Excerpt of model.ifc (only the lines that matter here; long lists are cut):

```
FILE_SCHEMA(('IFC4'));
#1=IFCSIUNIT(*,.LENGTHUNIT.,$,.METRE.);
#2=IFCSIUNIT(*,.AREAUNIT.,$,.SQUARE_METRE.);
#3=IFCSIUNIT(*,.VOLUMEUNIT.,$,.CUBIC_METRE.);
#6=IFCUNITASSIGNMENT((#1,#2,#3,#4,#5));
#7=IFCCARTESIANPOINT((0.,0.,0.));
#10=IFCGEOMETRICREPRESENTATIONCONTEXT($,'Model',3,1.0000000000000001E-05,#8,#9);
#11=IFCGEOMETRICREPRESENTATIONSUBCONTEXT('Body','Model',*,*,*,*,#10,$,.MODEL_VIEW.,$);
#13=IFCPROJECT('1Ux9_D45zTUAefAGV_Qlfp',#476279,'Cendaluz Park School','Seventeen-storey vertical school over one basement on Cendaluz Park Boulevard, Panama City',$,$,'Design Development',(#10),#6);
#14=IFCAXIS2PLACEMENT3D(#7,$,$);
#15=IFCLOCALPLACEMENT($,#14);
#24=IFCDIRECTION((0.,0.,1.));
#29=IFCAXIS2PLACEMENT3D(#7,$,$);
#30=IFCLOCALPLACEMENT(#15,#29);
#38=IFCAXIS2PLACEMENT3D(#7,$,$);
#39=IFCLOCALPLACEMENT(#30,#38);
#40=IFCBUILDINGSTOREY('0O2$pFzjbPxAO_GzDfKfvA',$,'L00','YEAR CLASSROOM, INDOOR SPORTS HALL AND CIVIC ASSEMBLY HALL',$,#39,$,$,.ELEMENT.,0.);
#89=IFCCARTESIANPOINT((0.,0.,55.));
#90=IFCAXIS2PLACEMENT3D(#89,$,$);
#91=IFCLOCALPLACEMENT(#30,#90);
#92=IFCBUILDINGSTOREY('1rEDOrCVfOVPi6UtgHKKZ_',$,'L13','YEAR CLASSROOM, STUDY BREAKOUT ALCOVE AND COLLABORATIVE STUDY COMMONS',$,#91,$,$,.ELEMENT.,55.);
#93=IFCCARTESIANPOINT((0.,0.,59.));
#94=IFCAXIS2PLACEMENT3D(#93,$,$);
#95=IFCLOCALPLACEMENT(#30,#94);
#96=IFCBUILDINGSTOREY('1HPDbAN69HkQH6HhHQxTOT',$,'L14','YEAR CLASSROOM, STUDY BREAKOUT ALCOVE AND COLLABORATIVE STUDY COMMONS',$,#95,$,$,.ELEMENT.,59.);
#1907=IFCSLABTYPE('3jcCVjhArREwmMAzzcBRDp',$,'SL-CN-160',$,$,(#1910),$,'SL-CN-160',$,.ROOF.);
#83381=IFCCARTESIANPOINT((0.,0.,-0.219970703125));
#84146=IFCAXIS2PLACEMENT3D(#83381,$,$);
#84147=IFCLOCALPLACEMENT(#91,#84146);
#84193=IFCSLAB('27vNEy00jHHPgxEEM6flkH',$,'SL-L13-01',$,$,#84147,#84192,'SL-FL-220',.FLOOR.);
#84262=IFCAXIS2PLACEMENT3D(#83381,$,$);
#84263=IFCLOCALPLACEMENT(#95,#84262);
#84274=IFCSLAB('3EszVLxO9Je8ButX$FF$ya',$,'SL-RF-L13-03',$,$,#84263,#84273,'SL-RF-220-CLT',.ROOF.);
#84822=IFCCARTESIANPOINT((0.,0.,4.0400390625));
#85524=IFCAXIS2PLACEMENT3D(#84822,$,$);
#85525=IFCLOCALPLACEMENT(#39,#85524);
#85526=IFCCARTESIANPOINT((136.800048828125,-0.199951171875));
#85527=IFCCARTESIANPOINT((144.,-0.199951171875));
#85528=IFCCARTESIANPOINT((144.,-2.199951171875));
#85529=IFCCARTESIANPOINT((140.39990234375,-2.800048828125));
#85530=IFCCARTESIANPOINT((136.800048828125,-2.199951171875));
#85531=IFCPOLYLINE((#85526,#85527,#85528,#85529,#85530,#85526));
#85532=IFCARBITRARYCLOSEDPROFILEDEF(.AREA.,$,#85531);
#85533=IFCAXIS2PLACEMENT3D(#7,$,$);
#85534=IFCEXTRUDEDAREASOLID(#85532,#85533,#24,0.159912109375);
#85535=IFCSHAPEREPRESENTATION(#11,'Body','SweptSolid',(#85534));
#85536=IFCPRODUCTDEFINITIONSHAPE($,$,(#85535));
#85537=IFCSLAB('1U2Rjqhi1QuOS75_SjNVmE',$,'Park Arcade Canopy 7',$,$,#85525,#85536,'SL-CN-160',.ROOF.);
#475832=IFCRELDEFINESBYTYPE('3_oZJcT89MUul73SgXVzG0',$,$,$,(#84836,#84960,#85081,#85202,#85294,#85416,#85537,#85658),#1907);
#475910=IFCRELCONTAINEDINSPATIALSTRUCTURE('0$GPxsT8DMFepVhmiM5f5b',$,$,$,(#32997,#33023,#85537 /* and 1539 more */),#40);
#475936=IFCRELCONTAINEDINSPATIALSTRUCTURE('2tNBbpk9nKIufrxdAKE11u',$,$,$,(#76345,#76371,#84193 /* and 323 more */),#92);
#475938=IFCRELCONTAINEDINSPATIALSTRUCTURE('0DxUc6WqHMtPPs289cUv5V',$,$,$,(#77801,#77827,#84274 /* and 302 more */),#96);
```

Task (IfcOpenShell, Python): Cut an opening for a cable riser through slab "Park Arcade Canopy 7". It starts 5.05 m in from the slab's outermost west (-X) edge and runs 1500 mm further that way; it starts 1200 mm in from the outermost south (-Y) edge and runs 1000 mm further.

```python
import numpy as np
import ifcopenshell
import ifcopenshell.api.feature
import ifcopenshell.api.geometry
import ifcopenshell.api.root
import ifcopenshell.geom
import ifcopenshell.util.placement
import ifcopenshell.util.representation
import ifcopenshell.util.shape
import ifcopenshell.util.unit

model = ifcopenshell.open("model.ifc")
unit_scale = ifcopenshell.util.unit.calculate_unit_scale(model)
settings = ifcopenshell.geom.settings()


def volume(element):
    """Net volume in cubic metres, openings subtracted."""
    shape = ifcopenshell.geom.create_shape(settings, element)
    return ifcopenshell.util.shape.get_volume(shape.geometry)


slab = model.by_id(85537)
before = volume(slab)

# Extent in the slab's own axes, in metres. The edges named are its -X and -Y sides.
slab_shape = ifcopenshell.geom.create_shape(settings, slab)
vertices = ifcopenshell.util.shape.get_vertices(slab_shape.geometry)
x_min, y_min, bottom = vertices.min(axis=0)
top = vertices[:, 2].max()

opening = ifcopenshell.api.root.create_entity(model, ifc_class="IfcOpeningElement", name="Cable riser opening", predefined_type="OPENING")
context = ifcopenshell.util.representation.get_context(model, "Model", "Body", "MODEL_VIEW")
width, depth = 1.5, 1
outline = [(0.0, 0.0), (width, 0.0), (width, depth), (0.0, depth), (0.0, 0.0)]
# Overshoot both faces by 50 mm so the cut is clean.
shape = ifcopenshell.api.geometry.add_slab_representation(
    model, context=context, depth=top - bottom + 0.1, polyline=outline
)
ifcopenshell.api.geometry.assign_representation(model, product=opening, representation=shape)

matrix = ifcopenshell.util.placement.get_local_placement(slab.ObjectPlacement)
matrix[:, 3] = matrix @ np.append(np.array([x_min + 5.05, y_min + 1.2, bottom - 0.05]) / unit_scale, 1.0)
ifcopenshell.api.geometry.edit_object_placement(model, product=opening, matrix=matrix, is_si=False)
ifcopenshell.api.feature.add_feature(model, feature=opening, element=slab)

after = volume(slab)

print(f"slab volume {before:.3f} -> {after:.3f} m3")

model.write("model-out.ifc")
```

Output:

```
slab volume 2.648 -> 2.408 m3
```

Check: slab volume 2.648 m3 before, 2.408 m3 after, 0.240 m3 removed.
